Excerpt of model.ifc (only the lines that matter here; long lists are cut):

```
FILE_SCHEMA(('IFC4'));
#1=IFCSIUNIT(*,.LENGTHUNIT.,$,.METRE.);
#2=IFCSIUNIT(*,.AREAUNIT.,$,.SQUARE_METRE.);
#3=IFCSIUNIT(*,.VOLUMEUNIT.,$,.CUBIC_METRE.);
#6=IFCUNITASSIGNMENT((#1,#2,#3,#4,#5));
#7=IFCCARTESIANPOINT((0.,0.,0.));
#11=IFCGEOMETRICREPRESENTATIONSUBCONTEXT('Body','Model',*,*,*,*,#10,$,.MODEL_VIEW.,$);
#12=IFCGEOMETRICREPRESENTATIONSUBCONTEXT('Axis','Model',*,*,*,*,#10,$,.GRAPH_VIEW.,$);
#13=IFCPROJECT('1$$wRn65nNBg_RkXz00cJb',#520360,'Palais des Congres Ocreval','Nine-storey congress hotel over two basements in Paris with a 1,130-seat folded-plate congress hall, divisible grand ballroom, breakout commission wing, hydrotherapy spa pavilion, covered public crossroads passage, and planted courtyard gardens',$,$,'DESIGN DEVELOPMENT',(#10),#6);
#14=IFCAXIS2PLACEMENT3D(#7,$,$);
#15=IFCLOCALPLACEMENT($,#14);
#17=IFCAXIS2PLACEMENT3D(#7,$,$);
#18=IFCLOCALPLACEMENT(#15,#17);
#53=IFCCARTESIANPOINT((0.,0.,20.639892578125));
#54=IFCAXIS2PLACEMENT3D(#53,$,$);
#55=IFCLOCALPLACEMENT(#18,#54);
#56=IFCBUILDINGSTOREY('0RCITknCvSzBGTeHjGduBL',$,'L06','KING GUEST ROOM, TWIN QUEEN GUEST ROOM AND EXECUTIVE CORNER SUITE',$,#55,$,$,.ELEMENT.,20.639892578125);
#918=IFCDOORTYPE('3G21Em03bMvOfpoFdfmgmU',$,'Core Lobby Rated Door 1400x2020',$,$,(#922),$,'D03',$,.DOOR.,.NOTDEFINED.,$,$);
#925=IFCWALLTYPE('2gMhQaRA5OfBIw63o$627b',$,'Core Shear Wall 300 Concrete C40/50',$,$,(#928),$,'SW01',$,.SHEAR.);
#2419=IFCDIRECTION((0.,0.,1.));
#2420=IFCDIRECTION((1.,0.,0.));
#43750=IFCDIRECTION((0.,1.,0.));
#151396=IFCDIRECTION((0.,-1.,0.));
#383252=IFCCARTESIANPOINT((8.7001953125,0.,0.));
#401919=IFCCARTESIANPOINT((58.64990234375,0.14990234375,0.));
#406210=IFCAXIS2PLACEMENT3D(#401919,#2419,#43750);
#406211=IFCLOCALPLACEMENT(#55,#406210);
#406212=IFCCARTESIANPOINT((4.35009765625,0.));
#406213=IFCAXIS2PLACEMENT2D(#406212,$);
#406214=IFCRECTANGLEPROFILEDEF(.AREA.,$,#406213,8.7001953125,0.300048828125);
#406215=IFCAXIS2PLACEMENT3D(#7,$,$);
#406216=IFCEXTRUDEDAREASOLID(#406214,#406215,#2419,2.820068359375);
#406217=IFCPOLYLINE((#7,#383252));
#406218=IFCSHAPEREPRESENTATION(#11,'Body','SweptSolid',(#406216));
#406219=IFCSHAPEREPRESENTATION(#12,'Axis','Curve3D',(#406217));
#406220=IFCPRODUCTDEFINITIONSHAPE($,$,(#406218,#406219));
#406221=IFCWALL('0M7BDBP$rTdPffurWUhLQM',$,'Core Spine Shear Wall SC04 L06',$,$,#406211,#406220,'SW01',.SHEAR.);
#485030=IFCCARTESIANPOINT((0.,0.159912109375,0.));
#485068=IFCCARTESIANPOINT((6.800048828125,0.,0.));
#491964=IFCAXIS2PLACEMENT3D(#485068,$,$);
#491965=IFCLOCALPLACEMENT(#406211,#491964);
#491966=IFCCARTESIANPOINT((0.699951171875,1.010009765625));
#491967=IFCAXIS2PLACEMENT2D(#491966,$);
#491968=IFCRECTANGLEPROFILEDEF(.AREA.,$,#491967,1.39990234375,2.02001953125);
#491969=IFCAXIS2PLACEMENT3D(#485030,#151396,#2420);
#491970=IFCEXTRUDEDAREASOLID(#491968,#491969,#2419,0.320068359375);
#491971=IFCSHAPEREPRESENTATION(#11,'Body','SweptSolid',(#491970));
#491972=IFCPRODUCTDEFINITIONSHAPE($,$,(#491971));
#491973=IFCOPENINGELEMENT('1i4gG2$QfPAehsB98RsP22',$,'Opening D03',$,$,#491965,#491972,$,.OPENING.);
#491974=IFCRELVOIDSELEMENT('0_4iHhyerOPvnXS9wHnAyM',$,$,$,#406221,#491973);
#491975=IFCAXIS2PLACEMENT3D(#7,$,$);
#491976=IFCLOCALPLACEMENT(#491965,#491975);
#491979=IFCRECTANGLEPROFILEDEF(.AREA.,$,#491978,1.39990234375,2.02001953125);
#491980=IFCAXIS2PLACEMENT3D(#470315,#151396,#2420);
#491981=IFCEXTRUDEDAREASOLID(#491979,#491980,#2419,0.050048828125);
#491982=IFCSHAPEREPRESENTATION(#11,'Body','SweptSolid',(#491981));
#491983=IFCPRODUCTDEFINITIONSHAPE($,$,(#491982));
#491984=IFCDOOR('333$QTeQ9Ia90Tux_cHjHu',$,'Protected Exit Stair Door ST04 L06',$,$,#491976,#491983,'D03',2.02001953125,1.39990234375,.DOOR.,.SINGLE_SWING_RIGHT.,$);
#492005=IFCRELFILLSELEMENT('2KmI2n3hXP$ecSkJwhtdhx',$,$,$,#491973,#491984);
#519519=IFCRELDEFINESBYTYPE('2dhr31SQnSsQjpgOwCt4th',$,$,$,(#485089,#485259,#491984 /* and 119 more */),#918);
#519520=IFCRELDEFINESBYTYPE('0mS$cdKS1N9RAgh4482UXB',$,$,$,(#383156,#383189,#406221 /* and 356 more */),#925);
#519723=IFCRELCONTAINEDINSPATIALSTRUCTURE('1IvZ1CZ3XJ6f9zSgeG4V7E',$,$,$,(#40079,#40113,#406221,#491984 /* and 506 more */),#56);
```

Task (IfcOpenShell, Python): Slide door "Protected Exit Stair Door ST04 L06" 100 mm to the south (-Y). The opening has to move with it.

```python
import ifcopenshell
import ifcopenshell.api.geometry
import ifcopenshell.util.placement
import ifcopenshell.util.unit

model = ifcopenshell.open("model.ifc")
unit_scale = ifcopenshell.util.unit.calculate_unit_scale(model)

door = model.by_id(491984)
opening = door.FillsVoids[0].RelatingOpeningElement
wall = opening.VoidsElements[0].RelatingBuildingElement

wall_matrix = ifcopenshell.util.placement.get_local_placement(wall.ObjectPlacement)
shift = wall_matrix[:3, 0] * -0.1 / unit_scale
before = ifcopenshell.util.placement.get_local_placement(door.ObjectPlacement)[:3, 3].copy()

# The door is placed relative to its opening, so it follows when the opening moves.
matrix = ifcopenshell.util.placement.get_local_placement(opening.ObjectPlacement)
matrix[:3, 3] += shift
ifcopenshell.api.geometry.edit_object_placement(
    model, product=opening, matrix=matrix, is_si=False, should_transform_children=True
)

after = ifcopenshell.util.placement.get_local_placement(door.ObjectPlacement)[:3, 3]
print("door moved by", (after - before).round(3) + 0.0)

model.write("model_v2.ifc")
```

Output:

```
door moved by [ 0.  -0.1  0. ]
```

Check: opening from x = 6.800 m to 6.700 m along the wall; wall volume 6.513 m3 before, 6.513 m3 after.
